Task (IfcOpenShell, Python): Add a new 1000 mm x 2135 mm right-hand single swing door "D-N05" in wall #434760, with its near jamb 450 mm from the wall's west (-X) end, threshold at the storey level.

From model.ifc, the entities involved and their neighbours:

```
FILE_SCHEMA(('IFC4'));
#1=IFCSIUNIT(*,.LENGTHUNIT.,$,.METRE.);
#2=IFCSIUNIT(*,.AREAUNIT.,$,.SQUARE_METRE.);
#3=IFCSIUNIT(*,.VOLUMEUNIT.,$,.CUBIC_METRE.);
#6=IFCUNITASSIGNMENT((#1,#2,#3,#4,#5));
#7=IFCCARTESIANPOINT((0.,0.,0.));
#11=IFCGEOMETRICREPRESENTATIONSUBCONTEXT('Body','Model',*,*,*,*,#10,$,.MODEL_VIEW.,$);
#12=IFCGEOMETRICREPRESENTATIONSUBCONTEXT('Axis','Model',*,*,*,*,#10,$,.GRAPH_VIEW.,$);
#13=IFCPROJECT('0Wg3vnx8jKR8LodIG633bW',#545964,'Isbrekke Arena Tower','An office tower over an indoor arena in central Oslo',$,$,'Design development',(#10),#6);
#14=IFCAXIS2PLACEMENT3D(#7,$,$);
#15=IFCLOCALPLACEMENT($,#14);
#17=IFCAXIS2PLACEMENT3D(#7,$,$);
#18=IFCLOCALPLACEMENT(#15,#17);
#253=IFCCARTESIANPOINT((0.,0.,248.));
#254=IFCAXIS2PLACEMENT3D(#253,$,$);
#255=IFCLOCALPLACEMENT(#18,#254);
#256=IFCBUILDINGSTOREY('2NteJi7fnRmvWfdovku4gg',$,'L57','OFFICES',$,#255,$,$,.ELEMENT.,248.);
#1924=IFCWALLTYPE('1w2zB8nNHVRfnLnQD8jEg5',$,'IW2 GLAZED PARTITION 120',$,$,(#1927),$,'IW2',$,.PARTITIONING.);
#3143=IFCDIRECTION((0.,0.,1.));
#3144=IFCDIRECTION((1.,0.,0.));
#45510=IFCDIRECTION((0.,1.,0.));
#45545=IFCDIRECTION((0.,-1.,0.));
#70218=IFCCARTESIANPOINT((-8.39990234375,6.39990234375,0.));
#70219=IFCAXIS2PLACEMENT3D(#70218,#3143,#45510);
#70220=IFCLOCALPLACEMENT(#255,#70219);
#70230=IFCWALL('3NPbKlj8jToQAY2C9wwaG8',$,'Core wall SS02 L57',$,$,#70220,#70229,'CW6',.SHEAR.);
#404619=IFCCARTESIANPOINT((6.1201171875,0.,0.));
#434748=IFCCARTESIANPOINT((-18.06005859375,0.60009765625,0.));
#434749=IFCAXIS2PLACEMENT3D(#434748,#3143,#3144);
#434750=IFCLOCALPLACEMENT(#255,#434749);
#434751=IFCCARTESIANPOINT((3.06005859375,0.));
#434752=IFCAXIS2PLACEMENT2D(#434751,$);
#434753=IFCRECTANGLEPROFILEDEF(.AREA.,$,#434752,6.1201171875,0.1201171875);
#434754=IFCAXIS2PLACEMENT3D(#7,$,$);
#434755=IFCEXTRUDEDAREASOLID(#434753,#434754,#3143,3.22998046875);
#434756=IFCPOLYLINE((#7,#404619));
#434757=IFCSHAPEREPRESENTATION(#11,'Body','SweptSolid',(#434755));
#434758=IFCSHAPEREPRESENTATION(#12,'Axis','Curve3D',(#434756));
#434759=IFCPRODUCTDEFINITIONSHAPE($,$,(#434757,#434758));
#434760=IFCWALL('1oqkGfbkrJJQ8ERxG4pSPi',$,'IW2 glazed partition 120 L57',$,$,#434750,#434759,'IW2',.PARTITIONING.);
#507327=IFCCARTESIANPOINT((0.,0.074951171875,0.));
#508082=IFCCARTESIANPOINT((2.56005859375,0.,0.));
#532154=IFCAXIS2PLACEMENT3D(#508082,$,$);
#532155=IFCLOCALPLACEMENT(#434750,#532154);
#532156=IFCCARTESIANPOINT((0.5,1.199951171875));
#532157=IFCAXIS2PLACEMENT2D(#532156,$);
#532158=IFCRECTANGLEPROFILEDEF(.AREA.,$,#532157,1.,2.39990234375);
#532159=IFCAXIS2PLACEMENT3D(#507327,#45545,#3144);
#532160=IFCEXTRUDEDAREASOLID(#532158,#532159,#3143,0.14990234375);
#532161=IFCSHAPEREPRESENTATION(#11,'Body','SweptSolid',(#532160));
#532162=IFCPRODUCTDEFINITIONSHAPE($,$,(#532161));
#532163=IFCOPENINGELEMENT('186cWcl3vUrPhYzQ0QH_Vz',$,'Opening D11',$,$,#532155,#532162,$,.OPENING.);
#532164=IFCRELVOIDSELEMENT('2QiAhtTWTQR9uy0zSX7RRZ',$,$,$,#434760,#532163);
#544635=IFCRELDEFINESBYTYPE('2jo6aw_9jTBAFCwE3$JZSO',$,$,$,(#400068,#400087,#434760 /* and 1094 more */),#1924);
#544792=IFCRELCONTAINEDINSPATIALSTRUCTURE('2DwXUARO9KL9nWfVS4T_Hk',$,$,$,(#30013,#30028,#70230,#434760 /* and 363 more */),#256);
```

```python
import numpy as np
import ifcopenshell
import ifcopenshell.api.feature
import ifcopenshell.api.geometry
import ifcopenshell.api.root
import ifcopenshell.api.spatial
import ifcopenshell.geom
import ifcopenshell.util.element
import ifcopenshell.util.placement
import ifcopenshell.util.representation
import ifcopenshell.util.shape
import ifcopenshell.util.unit

model = ifcopenshell.open("model.ifc")
unit_scale = ifcopenshell.util.unit.calculate_unit_scale(model)
settings = ifcopenshell.geom.settings()


def volume(element):
    """Net volume in cubic metres, openings subtracted."""
    shape = ifcopenshell.geom.create_shape(settings, element)
    return ifcopenshell.util.shape.get_volume(shape.geometry)


wall = model.by_guid("1oqkGfbkrJJQ8ERxG4pSPi")
storey = ifcopenshell.util.element.get_container(wall, ifc_class="IfcBuildingStorey")
context = ifcopenshell.util.representation.get_context(model, "Model", "Body", "MODEL_VIEW")
before = volume(wall)

width, height, from_end, sill = 1, 2.135, 0.45, 0.0  # metres

# The wall runs along its own X axis, and the end named is its -X end.
wall_shape = ifcopenshell.geom.create_shape(settings, wall)
x, y, z = ifcopenshell.util.shape.get_vertices(wall_shape.geometry).T
start = x.min() + from_end
face, thickness = float(y.min()), float(y.max() - y.min())
wall_matrix = ifcopenshell.util.placement.get_local_placement(wall.ObjectPlacement)
level = ifcopenshell.util.placement.get_local_placement(storey.ObjectPlacement)[2, 3]


def in_wall(x, y):
    """Placement at x, y metres in the wall's axes, at sill height."""
    matrix = wall_matrix.copy()
    matrix[:, 3] = wall_matrix @ np.array([x / unit_scale, y / unit_scale, 0.0, 1.0])
    matrix[2, 3] = level + sill / unit_scale
    return matrix


# Opening: a box that overshoots both wall faces by 50 mm.
opening = ifcopenshell.api.root.create_entity(model, ifc_class="IfcOpeningElement", predefined_type="OPENING")
box = ifcopenshell.api.geometry.add_wall_representation(
    model, context=context, length=width, height=height, thickness=thickness + 0.1
)
ifcopenshell.api.geometry.assign_representation(model, product=opening, representation=box)
ifcopenshell.api.geometry.edit_object_placement(model, product=opening, matrix=in_wall(start, face - 0.05), is_si=False)
ifcopenshell.api.feature.add_feature(model, feature=opening, element=wall)

door = ifcopenshell.api.root.create_entity(model, ifc_class="IfcDoor", name="D-N05", predefined_type="DOOR")
door.OverallWidth, door.OverallHeight = width / unit_scale, height / unit_scale
door.OperationType = "SINGLE_SWING_RIGHT"
body = ifcopenshell.api.geometry.add_door_representation(
    model,
    context=context,
    overall_width=door.OverallWidth,
    overall_height=door.OverallHeight,
    operation_type="SINGLE_SWING_RIGHT",
    lining_properties={"LiningDepth": thickness / unit_scale, "ThresholdDepth": thickness / unit_scale},
)
ifcopenshell.api.geometry.assign_representation(model, product=door, representation=body)
ifcopenshell.api.spatial.assign_container(model, products=[door], relating_structure=storey)
ifcopenshell.api.feature.add_filling(model, opening=opening, element=door)

# The lining spans the wall, so the door starts at the wall face.
ifcopenshell.api.geometry.edit_object_placement(model, product=door, matrix=in_wall(start, face), is_si=False)

after = volume(wall)

print(f"wall volume {before:.3f} -> {after:.3f} m3")

model.write("model-out.ifc")
```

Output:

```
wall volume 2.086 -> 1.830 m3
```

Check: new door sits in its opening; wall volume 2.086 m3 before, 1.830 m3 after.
